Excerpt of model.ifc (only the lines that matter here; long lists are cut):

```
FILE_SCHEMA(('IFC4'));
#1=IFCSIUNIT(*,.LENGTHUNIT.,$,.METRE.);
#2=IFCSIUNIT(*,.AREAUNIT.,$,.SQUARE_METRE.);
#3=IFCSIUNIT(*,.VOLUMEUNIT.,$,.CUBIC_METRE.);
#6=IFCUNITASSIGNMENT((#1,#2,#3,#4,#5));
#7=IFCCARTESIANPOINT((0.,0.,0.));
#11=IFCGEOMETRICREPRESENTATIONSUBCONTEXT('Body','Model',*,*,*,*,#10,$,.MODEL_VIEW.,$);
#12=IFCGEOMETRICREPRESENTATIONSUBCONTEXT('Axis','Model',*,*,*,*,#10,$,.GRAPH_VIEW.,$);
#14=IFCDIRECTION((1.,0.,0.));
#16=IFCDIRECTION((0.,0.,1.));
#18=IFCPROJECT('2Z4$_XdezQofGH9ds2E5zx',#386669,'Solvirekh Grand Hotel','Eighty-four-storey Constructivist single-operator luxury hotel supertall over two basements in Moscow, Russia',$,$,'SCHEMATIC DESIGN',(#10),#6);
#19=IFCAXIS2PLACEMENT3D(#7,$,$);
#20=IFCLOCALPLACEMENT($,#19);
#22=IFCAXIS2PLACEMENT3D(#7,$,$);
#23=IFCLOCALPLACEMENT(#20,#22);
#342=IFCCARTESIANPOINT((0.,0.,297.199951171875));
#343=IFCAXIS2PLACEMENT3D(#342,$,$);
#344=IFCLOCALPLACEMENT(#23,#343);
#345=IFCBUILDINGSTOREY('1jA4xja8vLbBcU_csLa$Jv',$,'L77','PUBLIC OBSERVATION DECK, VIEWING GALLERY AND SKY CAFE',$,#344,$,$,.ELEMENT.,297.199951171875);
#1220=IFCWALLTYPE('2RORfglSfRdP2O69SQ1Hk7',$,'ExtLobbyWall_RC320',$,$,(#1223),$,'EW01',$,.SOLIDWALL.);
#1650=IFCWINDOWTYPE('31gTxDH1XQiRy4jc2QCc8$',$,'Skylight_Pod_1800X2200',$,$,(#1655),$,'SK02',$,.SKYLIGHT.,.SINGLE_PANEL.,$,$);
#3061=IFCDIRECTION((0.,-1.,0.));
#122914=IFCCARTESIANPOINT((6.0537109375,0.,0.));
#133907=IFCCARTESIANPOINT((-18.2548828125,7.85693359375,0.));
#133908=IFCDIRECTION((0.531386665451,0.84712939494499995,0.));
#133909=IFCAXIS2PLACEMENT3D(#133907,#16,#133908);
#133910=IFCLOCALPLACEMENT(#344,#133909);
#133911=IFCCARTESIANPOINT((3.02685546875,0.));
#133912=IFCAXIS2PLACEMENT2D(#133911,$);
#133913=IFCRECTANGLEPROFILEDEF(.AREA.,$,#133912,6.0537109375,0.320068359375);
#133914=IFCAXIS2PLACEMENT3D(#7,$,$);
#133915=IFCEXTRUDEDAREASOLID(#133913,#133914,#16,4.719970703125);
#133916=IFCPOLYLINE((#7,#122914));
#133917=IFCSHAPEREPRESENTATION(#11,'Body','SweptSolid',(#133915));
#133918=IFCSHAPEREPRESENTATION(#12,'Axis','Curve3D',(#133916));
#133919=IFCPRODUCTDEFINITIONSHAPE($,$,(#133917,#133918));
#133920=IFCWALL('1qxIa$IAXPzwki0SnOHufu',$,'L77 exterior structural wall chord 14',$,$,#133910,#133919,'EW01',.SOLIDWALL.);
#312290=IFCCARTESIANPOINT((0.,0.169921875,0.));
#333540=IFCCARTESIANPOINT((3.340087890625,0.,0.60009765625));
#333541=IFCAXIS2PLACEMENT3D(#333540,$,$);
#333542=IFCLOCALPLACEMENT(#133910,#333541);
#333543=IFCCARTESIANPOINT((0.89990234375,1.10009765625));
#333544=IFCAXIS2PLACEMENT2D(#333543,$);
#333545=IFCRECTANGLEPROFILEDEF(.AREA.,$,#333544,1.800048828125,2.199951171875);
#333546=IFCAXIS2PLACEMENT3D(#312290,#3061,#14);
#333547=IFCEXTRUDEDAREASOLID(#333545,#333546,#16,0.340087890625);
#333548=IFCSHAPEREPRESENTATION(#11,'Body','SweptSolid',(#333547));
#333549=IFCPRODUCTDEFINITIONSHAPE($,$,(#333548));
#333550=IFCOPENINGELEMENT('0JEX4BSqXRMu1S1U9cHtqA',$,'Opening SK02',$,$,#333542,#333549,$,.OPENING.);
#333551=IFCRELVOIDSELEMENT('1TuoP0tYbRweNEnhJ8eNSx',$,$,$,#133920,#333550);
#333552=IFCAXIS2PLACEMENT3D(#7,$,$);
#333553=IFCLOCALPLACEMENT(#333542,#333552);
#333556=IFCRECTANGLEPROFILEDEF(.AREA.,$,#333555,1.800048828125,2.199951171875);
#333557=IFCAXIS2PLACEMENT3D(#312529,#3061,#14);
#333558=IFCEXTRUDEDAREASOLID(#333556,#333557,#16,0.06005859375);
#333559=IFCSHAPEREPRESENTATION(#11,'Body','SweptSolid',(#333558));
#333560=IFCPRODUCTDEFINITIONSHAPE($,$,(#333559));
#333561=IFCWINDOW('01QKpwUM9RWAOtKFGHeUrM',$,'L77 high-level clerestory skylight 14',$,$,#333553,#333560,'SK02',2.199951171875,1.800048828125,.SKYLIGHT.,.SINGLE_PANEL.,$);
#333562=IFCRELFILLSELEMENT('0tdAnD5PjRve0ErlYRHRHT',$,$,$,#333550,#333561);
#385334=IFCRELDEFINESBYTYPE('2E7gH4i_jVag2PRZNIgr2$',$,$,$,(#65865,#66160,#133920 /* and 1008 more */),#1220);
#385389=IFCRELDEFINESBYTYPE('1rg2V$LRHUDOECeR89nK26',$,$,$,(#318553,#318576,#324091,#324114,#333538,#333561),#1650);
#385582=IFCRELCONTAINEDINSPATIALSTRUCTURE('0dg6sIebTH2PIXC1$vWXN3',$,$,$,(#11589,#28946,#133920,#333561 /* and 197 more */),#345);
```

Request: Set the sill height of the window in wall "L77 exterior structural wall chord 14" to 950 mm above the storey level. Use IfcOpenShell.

```python
import numpy as np
import ifcopenshell
import ifcopenshell.api.geometry
import ifcopenshell.geom
import ifcopenshell.util.element
import ifcopenshell.util.placement
import ifcopenshell.util.shape
import ifcopenshell.util.unit

model = ifcopenshell.open("model.ifc")
unit_scale = ifcopenshell.util.unit.calculate_unit_scale(model)

window = model.by_id(333561)
opening = window.FillsVoids[0].RelatingOpeningElement
storey = ifcopenshell.util.element.get_container(window, ifc_class="IfcBuildingStorey")
level = ifcopenshell.util.placement.get_local_placement(storey.ObjectPlacement)[2, 3]

# The opening's origin need not be at the sill, so measure its lowest point.
shape = ifcopenshell.geom.create_shape(ifcopenshell.geom.settings(), opening)
bottom = ifcopenshell.util.shape.get_shape_bottom_elevation(shape, shape.geometry) / unit_scale
dz = level + 0.95 / unit_scale - bottom

shift = np.array([0.0, 0.0, dz])
# The window is placed relative to its opening, so it follows when the opening moves.
matrix = ifcopenshell.util.placement.get_local_placement(opening.ObjectPlacement)
matrix[:3, 3] += shift
ifcopenshell.api.geometry.edit_object_placement(
    model, product=opening, matrix=matrix, is_si=False, should_transform_children=True
)

print(f"moved by {dz * unit_scale:+.3f} m")

model.write("model_edited.ifc")
```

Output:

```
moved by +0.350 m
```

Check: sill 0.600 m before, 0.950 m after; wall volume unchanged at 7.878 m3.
